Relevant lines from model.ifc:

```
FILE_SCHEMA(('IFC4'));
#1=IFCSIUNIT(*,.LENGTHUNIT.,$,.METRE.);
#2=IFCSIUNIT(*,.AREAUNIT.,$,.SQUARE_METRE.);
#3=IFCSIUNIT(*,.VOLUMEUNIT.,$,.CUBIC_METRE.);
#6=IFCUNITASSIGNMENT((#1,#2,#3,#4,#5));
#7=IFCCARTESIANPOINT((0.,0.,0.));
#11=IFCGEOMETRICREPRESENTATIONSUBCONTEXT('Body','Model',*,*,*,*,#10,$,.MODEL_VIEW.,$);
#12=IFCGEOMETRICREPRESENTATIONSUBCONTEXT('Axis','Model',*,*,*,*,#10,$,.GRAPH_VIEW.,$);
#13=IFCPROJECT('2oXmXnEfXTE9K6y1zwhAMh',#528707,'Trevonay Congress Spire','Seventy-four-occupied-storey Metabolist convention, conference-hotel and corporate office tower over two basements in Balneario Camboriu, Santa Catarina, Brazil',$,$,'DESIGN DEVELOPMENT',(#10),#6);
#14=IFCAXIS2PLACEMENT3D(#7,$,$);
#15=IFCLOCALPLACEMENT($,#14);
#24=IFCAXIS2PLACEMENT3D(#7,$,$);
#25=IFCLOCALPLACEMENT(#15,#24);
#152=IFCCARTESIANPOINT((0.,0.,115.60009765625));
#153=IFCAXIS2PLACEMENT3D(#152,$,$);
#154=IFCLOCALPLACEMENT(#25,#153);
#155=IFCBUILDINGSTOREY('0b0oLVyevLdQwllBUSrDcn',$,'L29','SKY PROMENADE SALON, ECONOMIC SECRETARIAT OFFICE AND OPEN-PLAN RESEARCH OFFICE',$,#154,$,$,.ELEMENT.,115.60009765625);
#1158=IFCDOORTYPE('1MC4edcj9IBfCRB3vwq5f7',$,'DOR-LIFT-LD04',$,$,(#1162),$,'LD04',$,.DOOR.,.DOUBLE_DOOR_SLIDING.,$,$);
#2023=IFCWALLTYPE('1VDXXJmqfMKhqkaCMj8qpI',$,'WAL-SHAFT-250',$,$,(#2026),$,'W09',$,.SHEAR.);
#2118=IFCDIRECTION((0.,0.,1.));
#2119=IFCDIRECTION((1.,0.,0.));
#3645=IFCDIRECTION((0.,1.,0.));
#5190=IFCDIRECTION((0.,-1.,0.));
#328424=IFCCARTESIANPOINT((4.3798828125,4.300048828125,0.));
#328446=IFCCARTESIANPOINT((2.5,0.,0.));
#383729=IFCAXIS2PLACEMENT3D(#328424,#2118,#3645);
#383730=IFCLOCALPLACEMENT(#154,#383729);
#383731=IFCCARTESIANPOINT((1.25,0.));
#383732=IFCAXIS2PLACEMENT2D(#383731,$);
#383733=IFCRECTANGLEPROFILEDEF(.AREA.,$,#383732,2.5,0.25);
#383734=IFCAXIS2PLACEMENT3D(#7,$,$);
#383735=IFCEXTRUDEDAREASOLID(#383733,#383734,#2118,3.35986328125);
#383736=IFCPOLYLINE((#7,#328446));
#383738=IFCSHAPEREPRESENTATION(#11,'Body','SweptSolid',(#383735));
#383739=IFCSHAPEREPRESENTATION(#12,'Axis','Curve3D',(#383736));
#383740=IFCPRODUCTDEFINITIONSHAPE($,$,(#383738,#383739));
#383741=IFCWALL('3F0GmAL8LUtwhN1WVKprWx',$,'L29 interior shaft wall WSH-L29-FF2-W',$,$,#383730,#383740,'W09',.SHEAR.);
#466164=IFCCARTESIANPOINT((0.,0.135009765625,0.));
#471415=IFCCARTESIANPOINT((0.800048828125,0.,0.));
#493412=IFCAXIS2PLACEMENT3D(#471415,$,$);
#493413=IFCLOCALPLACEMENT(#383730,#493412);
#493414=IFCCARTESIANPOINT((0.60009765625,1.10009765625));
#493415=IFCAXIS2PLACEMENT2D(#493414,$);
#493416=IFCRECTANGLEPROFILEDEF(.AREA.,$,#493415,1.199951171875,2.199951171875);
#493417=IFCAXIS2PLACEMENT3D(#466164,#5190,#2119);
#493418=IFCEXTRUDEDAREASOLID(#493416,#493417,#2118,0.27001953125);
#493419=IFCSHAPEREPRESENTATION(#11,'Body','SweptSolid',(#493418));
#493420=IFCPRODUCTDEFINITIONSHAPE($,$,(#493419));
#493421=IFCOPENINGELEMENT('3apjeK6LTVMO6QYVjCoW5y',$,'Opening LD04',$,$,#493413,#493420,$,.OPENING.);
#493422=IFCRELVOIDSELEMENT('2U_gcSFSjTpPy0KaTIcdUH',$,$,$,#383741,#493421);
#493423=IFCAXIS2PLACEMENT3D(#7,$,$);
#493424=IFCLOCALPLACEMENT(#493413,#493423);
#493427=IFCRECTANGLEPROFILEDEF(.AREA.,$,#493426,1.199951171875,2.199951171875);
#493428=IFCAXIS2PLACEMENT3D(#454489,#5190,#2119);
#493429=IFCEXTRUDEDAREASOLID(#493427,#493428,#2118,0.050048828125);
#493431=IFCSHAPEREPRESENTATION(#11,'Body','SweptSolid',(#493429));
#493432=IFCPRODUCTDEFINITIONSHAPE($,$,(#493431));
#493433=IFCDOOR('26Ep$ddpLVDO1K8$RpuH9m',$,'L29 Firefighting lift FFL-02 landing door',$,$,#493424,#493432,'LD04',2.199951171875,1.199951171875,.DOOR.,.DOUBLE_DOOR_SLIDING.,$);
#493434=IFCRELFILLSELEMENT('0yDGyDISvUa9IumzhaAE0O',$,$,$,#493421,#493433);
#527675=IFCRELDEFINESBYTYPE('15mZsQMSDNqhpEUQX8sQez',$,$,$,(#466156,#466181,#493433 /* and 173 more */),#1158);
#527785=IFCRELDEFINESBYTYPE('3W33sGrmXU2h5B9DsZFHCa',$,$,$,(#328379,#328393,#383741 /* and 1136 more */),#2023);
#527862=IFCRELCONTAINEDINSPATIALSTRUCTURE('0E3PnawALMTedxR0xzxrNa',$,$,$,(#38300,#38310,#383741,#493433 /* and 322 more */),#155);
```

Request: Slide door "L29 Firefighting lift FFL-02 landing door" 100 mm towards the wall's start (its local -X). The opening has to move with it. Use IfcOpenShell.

```python
import ifcopenshell
import ifcopenshell.api.geometry
import ifcopenshell.util.placement
import ifcopenshell.util.unit

model = ifcopenshell.open("model.ifc")
unit_scale = ifcopenshell.util.unit.calculate_unit_scale(model)

door = model.by_guid("26Ep$ddpLVDO1K8$RpuH9m")
opening = door.FillsVoids[0].RelatingOpeningElement
wall = opening.VoidsElements[0].RelatingBuildingElement

wall_matrix = ifcopenshell.util.placement.get_local_placement(wall.ObjectPlacement)
shift = wall_matrix[:3, 0] * -0.1 / unit_scale
before = ifcopenshell.util.placement.get_local_placement(door.ObjectPlacement)[:3, 3].copy()

# The door is placed relative to its opening, so it follows when the opening moves.
matrix = ifcopenshell.util.placement.get_local_placement(opening.ObjectPlacement)
matrix[:3, 3] += shift
ifcopenshell.api.geometry.edit_object_placement(
    model, product=opening, matrix=matrix, is_si=False, should_transform_children=True
)

after = ifcopenshell.util.placement.get_local_placement(door.ObjectPlacement)[:3, 3]
print("door moved by", (after - before).round(3) + 0.0)

model.write("model_updated.ifc")
```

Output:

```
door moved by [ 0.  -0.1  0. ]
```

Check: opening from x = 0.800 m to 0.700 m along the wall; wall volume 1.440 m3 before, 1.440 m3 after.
